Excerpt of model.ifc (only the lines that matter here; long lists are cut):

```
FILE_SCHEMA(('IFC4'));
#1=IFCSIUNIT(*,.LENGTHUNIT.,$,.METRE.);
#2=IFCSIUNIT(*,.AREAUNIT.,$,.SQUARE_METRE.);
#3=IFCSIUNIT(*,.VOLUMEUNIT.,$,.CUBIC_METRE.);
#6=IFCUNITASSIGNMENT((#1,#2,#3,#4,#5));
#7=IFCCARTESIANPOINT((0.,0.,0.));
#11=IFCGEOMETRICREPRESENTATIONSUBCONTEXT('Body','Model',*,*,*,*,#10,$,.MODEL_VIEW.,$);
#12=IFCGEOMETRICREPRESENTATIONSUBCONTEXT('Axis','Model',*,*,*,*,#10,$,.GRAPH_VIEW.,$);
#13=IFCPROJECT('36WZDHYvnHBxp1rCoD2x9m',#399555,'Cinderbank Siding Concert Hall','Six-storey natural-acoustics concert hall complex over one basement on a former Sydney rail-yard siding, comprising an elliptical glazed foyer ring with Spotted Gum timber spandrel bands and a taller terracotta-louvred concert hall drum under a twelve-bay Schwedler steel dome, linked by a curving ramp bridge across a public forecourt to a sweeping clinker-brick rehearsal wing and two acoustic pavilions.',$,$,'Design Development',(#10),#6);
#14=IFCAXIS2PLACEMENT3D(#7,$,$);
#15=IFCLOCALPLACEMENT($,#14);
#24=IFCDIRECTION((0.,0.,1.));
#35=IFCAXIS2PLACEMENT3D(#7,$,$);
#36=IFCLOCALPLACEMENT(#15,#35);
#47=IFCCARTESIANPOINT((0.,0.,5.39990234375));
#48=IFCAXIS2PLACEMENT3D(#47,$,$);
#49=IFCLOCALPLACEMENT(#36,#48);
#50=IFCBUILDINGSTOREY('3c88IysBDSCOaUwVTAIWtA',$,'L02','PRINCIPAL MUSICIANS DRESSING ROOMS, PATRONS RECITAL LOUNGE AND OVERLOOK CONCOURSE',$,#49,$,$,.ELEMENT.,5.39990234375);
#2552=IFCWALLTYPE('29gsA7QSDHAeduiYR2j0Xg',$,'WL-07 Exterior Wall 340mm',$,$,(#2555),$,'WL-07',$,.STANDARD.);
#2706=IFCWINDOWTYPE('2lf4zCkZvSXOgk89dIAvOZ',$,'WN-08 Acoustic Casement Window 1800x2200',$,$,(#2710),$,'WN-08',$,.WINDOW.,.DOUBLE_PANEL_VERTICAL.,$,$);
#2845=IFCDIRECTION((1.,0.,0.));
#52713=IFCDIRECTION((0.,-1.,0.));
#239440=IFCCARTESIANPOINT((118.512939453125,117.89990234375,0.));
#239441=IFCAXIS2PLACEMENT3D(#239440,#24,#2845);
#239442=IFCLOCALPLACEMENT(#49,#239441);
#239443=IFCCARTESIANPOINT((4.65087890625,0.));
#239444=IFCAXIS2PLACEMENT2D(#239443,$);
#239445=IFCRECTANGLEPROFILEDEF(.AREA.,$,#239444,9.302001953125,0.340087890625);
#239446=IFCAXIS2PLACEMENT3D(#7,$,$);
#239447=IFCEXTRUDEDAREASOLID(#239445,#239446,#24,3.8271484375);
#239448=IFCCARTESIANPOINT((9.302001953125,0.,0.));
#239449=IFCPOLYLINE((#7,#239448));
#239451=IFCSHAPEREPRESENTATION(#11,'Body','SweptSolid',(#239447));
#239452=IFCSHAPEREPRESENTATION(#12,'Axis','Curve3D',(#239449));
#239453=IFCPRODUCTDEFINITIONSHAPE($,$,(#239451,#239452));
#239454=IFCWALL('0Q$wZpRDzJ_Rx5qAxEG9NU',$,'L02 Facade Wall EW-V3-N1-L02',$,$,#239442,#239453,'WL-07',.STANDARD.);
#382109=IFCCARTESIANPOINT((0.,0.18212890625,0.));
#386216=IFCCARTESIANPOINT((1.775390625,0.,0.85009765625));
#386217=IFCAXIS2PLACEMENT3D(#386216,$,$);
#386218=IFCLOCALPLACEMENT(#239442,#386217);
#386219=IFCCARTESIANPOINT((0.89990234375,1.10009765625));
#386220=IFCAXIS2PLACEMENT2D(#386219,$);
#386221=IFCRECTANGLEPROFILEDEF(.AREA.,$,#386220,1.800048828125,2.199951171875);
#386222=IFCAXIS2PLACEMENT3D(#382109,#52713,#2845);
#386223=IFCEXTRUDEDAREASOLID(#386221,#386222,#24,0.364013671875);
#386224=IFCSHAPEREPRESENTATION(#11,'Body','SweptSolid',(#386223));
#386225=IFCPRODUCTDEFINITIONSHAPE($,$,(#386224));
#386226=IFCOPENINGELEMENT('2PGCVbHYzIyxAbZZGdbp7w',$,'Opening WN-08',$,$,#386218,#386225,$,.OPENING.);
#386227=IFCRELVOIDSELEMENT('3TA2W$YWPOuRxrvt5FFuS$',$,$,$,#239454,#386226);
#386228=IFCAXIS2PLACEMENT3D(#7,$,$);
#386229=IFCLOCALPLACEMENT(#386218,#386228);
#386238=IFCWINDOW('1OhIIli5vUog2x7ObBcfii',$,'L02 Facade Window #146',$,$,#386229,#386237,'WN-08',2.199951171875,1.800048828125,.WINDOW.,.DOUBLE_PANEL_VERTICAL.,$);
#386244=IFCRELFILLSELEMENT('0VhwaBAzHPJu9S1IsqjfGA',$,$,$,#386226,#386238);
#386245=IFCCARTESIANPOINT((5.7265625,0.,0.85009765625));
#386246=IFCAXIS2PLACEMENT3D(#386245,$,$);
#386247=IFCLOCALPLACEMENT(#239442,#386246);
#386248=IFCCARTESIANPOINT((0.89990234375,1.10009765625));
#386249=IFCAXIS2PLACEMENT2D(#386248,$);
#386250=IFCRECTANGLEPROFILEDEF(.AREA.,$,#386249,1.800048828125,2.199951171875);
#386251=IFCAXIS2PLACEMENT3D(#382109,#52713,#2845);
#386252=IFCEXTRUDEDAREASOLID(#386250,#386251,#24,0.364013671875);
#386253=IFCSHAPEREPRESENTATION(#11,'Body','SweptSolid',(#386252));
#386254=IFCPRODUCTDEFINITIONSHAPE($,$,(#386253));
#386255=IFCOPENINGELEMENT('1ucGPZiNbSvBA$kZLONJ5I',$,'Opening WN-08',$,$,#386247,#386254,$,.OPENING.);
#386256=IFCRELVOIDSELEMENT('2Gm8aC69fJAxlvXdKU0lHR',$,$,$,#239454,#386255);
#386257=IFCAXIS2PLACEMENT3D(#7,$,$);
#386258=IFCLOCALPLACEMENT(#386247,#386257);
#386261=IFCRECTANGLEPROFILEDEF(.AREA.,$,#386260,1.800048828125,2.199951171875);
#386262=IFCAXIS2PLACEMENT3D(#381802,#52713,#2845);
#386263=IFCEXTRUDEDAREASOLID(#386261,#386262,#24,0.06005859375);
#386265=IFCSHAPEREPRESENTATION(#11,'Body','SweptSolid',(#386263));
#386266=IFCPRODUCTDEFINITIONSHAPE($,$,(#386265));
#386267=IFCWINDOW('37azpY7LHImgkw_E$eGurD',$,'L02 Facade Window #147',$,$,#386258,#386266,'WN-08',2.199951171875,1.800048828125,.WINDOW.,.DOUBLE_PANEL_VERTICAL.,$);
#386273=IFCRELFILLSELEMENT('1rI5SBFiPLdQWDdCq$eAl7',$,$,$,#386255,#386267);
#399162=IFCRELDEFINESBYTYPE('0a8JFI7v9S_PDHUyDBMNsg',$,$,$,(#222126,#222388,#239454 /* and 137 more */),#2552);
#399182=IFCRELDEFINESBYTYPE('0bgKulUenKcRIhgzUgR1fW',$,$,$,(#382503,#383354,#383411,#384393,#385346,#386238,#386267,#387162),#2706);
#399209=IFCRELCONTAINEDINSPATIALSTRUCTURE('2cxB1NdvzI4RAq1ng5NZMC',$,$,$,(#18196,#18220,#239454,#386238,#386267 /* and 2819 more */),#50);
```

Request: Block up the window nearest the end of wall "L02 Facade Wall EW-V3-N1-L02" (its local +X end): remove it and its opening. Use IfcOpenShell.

```python
import ifcopenshell
import ifcopenshell.api.feature
import ifcopenshell.api.root
import ifcopenshell.geom
import ifcopenshell.util.shape

model = ifcopenshell.open("model.ifc")
settings = ifcopenshell.geom.settings()


def volume(element):
    """Net volume in cubic metres, openings subtracted."""
    shape = ifcopenshell.geom.create_shape(settings, element)
    return ifcopenshell.util.shape.get_volume(shape.geometry)


window = model.by_id(386267)
opening = window.FillsVoids[0].RelatingOpeningElement
wall = opening.VoidsElements[0].RelatingBuildingElement
before = volume(wall)

ifcopenshell.api.root.remove_product(model, product=window)
ifcopenshell.api.feature.remove_feature(model, feature=opening)

after = volume(wall)

print(f"wall volume {before:.3f} -> {after:.3f} m3")

model.write("model_v2.ifc")
```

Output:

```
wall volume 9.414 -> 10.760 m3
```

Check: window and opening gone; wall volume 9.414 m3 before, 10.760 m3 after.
